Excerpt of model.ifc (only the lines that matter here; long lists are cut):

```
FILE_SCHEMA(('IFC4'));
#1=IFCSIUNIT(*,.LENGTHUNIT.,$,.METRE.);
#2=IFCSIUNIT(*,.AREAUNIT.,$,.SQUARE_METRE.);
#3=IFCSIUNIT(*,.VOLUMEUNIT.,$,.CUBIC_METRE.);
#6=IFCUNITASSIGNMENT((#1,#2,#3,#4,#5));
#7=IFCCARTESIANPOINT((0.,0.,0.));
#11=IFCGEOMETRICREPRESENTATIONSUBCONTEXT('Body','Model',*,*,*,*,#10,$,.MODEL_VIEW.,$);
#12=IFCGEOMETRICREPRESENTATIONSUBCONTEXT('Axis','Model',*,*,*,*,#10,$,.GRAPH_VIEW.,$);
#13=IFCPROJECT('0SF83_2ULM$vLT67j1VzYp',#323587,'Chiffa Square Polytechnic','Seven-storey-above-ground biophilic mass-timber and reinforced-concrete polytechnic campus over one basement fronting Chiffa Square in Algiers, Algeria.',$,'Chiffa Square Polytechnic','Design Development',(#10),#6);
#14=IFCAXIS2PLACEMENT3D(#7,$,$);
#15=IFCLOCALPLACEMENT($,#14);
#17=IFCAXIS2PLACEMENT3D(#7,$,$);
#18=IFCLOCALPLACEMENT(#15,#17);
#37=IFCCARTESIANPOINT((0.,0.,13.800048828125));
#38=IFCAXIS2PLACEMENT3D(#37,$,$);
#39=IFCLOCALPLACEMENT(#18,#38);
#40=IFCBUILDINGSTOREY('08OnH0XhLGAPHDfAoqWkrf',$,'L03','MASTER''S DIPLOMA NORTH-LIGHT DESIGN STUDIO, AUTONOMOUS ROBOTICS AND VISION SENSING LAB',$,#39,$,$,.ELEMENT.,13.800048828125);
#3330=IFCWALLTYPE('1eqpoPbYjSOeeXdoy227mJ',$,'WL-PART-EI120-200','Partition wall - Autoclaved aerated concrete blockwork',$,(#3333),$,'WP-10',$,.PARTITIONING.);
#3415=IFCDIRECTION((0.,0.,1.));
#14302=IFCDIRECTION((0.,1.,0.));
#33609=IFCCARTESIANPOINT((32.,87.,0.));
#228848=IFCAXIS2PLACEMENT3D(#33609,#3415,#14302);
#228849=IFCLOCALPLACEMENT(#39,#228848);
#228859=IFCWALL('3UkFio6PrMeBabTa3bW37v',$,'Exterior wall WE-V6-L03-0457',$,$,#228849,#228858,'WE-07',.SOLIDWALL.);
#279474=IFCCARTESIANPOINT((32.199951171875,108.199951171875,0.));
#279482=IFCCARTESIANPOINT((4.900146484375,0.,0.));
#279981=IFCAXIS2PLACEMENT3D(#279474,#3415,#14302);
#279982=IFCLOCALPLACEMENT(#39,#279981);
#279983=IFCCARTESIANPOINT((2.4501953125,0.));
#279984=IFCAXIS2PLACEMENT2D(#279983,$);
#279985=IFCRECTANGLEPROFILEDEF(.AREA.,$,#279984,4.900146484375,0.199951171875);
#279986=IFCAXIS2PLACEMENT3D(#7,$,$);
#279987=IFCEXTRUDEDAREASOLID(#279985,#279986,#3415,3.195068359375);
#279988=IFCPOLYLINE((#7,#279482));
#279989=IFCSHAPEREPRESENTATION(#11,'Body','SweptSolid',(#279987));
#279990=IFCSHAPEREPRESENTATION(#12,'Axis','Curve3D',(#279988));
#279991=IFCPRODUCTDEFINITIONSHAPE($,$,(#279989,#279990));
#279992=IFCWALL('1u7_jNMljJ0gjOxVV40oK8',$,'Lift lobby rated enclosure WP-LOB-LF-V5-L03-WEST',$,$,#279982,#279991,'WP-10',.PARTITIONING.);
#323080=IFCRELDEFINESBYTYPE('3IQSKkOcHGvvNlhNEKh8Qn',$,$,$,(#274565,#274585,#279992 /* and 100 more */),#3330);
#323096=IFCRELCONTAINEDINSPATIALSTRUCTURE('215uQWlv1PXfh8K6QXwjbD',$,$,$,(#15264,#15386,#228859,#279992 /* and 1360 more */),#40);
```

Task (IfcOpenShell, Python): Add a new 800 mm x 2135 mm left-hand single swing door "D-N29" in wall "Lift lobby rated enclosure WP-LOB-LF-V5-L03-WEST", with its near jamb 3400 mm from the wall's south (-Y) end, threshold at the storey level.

```python
import numpy as np
import ifcopenshell
import ifcopenshell.api.feature
import ifcopenshell.api.geometry
import ifcopenshell.api.root
import ifcopenshell.api.spatial
import ifcopenshell.geom
import ifcopenshell.util.element
import ifcopenshell.util.placement
import ifcopenshell.util.representation
import ifcopenshell.util.shape
import ifcopenshell.util.unit

model = ifcopenshell.open("model.ifc")
unit_scale = ifcopenshell.util.unit.calculate_unit_scale(model)
settings = ifcopenshell.geom.settings()


def volume(element):
    """Net volume in cubic metres, openings subtracted."""
    shape = ifcopenshell.geom.create_shape(settings, element)
    return ifcopenshell.util.shape.get_volume(shape.geometry)


wall = model.by_id(279992)
storey = ifcopenshell.util.element.get_container(wall, ifc_class="IfcBuildingStorey")
context = ifcopenshell.util.representation.get_context(model, "Model", "Body", "MODEL_VIEW")
before = volume(wall)

width, height, from_end, sill = 0.8, 2.135, 3.4, 0.0  # metres

# The wall runs along its own X axis, and the end named is its -X end.
wall_shape = ifcopenshell.geom.create_shape(settings, wall)
x, y, z = ifcopenshell.util.shape.get_vertices(wall_shape.geometry).T
start = x.min() + from_end
face, thickness = float(y.min()), float(y.max() - y.min())
wall_matrix = ifcopenshell.util.placement.get_local_placement(wall.ObjectPlacement)
level = ifcopenshell.util.placement.get_local_placement(storey.ObjectPlacement)[2, 3]


def in_wall(x, y):
    """Placement at x, y metres in the wall's axes, at sill height."""
    matrix = wall_matrix.copy()
    matrix[:, 3] = wall_matrix @ np.array([x / unit_scale, y / unit_scale, 0.0, 1.0])
    matrix[2, 3] = level + sill / unit_scale
    return matrix


# Opening: a box that overshoots both wall faces by 50 mm.
opening = ifcopenshell.api.root.create_entity(model, ifc_class="IfcOpeningElement", predefined_type="OPENING")
box = ifcopenshell.api.geometry.add_wall_representation(
    model, context=context, length=width, height=height, thickness=thickness + 0.1
)
ifcopenshell.api.geometry.assign_representation(model, product=opening, representation=box)
ifcopenshell.api.geometry.edit_object_placement(model, product=opening, matrix=in_wall(start, face - 0.05), is_si=False)
ifcopenshell.api.feature.add_feature(model, feature=opening, element=wall)

door = ifcopenshell.api.root.create_entity(model, ifc_class="IfcDoor", name="D-N29", predefined_type="DOOR")
door.OverallWidth, door.OverallHeight = width / unit_scale, height / unit_scale
door.OperationType = "SINGLE_SWING_LEFT"
body = ifcopenshell.api.geometry.add_door_representation(
    model,
    context=context,
    overall_width=door.OverallWidth,
    overall_height=door.OverallHeight,
    operation_type="SINGLE_SWING_LEFT",
    lining_properties={"LiningDepth": thickness / unit_scale, "ThresholdDepth": thickness / unit_scale},
)
ifcopenshell.api.geometry.assign_representation(model, product=door, representation=body)
ifcopenshell.api.spatial.assign_container(model, products=[door], relating_structure=storey)
ifcopenshell.api.feature.add_filling(model, opening=opening, element=door)

# The lining spans the wall, so the door starts at the wall face.
ifcopenshell.api.geometry.edit_object_placement(model, product=door, matrix=in_wall(start, face), is_si=False)

after = volume(wall)

print(f"wall volume {before:.3f} -> {after:.3f} m3")

model.write("model_rev.ifc")
```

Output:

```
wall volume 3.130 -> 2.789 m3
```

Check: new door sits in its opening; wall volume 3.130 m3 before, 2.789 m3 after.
